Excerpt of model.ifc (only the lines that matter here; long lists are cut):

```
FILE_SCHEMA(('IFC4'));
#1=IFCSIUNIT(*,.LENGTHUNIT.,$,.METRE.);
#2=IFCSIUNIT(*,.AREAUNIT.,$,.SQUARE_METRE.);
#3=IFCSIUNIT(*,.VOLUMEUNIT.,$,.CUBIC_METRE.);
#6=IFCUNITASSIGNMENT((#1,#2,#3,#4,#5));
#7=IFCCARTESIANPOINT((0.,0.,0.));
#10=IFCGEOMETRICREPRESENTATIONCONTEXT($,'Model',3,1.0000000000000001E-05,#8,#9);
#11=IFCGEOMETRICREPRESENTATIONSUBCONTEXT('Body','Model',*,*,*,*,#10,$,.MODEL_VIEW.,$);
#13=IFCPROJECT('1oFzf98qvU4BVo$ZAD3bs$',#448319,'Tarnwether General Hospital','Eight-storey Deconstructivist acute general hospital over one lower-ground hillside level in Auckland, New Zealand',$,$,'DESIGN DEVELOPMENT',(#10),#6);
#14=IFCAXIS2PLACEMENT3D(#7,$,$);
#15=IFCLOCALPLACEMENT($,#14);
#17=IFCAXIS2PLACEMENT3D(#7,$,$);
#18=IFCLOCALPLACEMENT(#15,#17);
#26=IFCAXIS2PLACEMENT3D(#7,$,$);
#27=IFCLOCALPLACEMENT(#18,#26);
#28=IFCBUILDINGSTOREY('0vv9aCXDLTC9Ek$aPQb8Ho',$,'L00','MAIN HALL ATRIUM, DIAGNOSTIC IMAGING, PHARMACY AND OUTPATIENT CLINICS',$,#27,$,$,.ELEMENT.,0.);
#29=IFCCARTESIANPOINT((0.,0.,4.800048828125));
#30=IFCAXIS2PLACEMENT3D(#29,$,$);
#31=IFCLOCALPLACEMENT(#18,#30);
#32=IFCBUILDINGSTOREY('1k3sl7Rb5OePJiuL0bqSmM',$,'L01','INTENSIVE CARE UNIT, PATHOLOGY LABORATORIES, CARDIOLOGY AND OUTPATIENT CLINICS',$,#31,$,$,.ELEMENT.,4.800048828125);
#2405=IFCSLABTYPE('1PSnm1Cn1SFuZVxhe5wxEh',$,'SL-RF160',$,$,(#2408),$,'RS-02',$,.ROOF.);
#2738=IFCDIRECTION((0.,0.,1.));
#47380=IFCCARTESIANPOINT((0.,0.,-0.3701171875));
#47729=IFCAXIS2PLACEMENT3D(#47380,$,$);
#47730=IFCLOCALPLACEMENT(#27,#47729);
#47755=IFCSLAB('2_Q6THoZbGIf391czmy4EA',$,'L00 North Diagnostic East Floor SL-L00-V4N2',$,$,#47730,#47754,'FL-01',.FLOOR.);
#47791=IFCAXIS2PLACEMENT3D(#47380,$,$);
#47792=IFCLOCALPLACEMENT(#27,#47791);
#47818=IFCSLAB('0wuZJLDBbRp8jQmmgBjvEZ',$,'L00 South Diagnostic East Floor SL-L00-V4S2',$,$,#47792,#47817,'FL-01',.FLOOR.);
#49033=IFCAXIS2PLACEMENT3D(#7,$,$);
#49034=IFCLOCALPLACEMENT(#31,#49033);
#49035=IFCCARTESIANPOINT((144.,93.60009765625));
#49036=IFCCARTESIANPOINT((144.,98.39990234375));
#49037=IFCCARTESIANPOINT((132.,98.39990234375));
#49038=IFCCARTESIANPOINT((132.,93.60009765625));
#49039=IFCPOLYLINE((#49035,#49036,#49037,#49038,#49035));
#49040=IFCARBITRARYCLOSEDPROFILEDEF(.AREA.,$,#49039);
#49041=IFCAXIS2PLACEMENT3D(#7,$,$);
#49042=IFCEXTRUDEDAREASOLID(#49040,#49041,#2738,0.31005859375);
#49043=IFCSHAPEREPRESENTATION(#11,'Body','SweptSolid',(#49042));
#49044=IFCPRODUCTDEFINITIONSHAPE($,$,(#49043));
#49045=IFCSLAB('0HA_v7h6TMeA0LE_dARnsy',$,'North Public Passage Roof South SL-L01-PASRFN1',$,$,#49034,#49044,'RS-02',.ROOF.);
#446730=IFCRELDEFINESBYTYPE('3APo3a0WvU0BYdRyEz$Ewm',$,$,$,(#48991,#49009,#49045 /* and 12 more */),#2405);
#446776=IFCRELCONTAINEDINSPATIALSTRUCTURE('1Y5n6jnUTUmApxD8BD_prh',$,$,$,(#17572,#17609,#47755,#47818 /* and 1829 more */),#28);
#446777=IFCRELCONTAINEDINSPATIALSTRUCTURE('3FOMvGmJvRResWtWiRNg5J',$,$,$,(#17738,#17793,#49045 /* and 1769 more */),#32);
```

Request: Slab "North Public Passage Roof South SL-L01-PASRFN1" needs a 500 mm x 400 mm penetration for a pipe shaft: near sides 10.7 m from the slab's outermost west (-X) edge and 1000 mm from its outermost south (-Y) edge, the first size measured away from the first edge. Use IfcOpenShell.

```python
import numpy as np
import ifcopenshell
import ifcopenshell.api.feature
import ifcopenshell.api.geometry
import ifcopenshell.api.root
import ifcopenshell.geom
import ifcopenshell.util.placement
import ifcopenshell.util.representation
import ifcopenshell.util.shape
import ifcopenshell.util.unit

model = ifcopenshell.open("model.ifc")
unit_scale = ifcopenshell.util.unit.calculate_unit_scale(model)
settings = ifcopenshell.geom.settings()


def volume(element):
    """Net volume in cubic metres, openings subtracted."""
    shape = ifcopenshell.geom.create_shape(settings, element)
    return ifcopenshell.util.shape.get_volume(shape.geometry)


slab = model.by_guid("0HA_v7h6TMeA0LE_dARnsy")
before = volume(slab)

# Extent in the slab's own axes, in metres. The edges named are its -X and -Y sides.
slab_shape = ifcopenshell.geom.create_shape(settings, slab)
vertices = ifcopenshell.util.shape.get_vertices(slab_shape.geometry)
x_min, y_min, bottom = vertices.min(axis=0)
top = vertices[:, 2].max()

opening = ifcopenshell.api.root.create_entity(model, ifc_class="IfcOpeningElement", name="Pipe shaft opening", predefined_type="OPENING")
context = ifcopenshell.util.representation.get_context(model, "Model", "Body", "MODEL_VIEW")
width, depth = 0.5, 0.4
outline = [(0.0, 0.0), (width, 0.0), (width, depth), (0.0, depth), (0.0, 0.0)]
# Overshoot both faces by 50 mm so the cut is clean.
shape = ifcopenshell.api.geometry.add_slab_representation(
    model, context=context, depth=top - bottom + 0.1, polyline=outline
)
ifcopenshell.api.geometry.assign_representation(model, product=opening, representation=shape)

matrix = ifcopenshell.util.placement.get_local_placement(slab.ObjectPlacement)
matrix[:, 3] = matrix @ np.append(np.array([x_min + 10.7, y_min + 1, bottom - 0.05]) / unit_scale, 1.0)
ifcopenshell.api.geometry.edit_object_placement(model, product=opening, matrix=matrix, is_si=False)
ifcopenshell.api.feature.add_feature(model, feature=opening, element=slab)

after = volume(slab)

print(f"slab volume {before:.3f} -> {after:.3f} m3")

model.write("model_v2.ifc")
```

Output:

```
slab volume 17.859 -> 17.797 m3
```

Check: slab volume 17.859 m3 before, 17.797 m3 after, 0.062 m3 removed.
